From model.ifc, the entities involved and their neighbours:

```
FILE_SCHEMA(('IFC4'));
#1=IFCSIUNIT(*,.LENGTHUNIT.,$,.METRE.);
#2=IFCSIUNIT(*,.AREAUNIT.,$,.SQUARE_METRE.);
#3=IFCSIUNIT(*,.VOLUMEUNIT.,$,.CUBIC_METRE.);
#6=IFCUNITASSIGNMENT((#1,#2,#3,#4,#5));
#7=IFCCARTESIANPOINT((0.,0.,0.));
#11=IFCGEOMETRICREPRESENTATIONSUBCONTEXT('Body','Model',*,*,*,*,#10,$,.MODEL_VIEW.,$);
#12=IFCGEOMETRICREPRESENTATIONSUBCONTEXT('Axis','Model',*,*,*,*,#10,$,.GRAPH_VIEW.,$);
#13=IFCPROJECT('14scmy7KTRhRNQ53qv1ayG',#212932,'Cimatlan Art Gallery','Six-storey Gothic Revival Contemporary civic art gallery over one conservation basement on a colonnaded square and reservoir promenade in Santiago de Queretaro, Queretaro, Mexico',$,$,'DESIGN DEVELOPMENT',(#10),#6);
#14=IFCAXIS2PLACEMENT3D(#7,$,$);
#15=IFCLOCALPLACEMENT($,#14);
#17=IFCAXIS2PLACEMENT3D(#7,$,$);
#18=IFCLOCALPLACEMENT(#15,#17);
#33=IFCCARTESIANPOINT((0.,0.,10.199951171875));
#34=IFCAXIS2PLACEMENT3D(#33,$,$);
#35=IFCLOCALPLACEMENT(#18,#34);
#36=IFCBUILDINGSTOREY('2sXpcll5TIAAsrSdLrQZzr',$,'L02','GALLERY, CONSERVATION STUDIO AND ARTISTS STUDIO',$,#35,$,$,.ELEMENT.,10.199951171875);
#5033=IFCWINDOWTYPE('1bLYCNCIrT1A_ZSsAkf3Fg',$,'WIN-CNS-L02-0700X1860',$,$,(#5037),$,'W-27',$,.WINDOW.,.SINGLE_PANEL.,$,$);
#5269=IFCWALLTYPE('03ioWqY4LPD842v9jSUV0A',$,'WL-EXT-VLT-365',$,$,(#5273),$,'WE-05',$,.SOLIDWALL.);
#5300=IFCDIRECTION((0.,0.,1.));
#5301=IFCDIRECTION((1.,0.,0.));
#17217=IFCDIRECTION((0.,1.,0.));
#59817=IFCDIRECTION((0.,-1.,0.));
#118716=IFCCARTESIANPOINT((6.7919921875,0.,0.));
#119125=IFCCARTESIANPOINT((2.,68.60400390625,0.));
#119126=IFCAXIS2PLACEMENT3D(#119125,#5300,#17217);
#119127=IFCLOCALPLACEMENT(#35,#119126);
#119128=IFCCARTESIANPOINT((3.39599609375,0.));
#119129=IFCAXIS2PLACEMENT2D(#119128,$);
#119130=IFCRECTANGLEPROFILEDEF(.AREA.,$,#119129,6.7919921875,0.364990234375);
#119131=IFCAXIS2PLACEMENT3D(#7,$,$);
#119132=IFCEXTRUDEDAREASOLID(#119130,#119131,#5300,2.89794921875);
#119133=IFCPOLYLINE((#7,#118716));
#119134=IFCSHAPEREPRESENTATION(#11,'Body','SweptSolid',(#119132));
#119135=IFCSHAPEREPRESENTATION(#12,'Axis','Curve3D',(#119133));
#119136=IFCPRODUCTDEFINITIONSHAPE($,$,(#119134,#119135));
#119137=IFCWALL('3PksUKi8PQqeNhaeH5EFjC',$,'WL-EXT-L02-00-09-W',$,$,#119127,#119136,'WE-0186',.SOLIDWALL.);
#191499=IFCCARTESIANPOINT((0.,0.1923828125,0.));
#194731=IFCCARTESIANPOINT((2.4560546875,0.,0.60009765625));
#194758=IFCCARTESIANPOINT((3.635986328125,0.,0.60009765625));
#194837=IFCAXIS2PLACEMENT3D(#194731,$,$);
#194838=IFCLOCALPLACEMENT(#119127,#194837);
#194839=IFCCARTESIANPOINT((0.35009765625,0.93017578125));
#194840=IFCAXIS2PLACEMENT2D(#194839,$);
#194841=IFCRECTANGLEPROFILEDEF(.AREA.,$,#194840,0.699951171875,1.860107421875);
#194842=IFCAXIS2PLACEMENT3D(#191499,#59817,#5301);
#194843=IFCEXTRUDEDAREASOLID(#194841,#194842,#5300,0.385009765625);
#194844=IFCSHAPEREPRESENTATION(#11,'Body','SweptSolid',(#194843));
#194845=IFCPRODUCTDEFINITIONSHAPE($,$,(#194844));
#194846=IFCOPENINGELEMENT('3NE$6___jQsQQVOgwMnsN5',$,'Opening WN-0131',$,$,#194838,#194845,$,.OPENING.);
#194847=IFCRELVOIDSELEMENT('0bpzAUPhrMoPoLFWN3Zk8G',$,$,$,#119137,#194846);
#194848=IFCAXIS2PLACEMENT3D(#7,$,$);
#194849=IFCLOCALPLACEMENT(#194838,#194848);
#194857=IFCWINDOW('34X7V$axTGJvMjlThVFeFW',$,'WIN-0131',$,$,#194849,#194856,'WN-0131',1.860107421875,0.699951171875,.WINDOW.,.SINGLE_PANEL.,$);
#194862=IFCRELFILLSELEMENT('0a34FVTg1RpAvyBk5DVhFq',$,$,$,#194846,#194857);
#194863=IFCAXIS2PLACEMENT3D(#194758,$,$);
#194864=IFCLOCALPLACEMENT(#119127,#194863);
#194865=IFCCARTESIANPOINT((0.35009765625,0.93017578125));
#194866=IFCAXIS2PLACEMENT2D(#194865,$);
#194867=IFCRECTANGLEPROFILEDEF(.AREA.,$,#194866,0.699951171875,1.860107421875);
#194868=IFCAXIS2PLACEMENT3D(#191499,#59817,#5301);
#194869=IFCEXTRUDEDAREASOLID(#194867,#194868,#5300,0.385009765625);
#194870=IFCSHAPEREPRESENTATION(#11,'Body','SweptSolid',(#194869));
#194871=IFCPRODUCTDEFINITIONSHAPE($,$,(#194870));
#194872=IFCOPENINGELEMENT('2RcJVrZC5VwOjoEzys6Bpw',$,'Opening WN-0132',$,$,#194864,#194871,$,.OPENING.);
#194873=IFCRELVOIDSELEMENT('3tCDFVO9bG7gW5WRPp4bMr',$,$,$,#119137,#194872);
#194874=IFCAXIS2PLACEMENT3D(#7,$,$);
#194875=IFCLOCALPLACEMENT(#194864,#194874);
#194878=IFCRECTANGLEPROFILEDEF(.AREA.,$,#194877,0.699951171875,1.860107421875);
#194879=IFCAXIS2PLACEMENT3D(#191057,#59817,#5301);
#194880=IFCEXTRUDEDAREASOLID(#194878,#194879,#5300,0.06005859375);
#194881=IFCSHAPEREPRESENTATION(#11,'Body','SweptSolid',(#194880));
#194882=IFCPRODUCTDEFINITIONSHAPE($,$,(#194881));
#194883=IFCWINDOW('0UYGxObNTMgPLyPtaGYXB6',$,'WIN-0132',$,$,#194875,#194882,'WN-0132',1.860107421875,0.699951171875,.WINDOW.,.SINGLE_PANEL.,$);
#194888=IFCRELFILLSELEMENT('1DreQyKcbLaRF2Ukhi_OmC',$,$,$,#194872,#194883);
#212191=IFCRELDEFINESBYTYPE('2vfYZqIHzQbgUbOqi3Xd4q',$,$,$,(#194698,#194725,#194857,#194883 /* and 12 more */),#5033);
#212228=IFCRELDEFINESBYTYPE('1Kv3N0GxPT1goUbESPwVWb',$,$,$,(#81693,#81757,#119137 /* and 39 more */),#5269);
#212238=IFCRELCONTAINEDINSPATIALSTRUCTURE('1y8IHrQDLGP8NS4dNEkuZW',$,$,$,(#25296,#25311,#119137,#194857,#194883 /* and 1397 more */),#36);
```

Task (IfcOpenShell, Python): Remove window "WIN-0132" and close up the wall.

```python
import ifcopenshell
import ifcopenshell.api.feature
import ifcopenshell.api.root
import ifcopenshell.geom
import ifcopenshell.util.shape

model = ifcopenshell.open("model.ifc")
settings = ifcopenshell.geom.settings()


def volume(element):
    """Net volume in cubic metres, openings subtracted."""
    shape = ifcopenshell.geom.create_shape(settings, element)
    return ifcopenshell.util.shape.get_volume(shape.geometry)


window = model.by_guid("0UYGxObNTMgPLyPtaGYXB6")
opening = window.FillsVoids[0].RelatingOpeningElement
wall = opening.VoidsElements[0].RelatingBuildingElement
before = volume(wall)

ifcopenshell.api.root.remove_product(model, product=window)
ifcopenshell.api.feature.remove_feature(model, feature=opening)

after = volume(wall)

print(f"wall volume {before:.3f} -> {after:.3f} m3")

model.write("model_v2.ifc")
```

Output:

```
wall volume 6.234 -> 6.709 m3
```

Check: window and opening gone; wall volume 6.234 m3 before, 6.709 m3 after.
